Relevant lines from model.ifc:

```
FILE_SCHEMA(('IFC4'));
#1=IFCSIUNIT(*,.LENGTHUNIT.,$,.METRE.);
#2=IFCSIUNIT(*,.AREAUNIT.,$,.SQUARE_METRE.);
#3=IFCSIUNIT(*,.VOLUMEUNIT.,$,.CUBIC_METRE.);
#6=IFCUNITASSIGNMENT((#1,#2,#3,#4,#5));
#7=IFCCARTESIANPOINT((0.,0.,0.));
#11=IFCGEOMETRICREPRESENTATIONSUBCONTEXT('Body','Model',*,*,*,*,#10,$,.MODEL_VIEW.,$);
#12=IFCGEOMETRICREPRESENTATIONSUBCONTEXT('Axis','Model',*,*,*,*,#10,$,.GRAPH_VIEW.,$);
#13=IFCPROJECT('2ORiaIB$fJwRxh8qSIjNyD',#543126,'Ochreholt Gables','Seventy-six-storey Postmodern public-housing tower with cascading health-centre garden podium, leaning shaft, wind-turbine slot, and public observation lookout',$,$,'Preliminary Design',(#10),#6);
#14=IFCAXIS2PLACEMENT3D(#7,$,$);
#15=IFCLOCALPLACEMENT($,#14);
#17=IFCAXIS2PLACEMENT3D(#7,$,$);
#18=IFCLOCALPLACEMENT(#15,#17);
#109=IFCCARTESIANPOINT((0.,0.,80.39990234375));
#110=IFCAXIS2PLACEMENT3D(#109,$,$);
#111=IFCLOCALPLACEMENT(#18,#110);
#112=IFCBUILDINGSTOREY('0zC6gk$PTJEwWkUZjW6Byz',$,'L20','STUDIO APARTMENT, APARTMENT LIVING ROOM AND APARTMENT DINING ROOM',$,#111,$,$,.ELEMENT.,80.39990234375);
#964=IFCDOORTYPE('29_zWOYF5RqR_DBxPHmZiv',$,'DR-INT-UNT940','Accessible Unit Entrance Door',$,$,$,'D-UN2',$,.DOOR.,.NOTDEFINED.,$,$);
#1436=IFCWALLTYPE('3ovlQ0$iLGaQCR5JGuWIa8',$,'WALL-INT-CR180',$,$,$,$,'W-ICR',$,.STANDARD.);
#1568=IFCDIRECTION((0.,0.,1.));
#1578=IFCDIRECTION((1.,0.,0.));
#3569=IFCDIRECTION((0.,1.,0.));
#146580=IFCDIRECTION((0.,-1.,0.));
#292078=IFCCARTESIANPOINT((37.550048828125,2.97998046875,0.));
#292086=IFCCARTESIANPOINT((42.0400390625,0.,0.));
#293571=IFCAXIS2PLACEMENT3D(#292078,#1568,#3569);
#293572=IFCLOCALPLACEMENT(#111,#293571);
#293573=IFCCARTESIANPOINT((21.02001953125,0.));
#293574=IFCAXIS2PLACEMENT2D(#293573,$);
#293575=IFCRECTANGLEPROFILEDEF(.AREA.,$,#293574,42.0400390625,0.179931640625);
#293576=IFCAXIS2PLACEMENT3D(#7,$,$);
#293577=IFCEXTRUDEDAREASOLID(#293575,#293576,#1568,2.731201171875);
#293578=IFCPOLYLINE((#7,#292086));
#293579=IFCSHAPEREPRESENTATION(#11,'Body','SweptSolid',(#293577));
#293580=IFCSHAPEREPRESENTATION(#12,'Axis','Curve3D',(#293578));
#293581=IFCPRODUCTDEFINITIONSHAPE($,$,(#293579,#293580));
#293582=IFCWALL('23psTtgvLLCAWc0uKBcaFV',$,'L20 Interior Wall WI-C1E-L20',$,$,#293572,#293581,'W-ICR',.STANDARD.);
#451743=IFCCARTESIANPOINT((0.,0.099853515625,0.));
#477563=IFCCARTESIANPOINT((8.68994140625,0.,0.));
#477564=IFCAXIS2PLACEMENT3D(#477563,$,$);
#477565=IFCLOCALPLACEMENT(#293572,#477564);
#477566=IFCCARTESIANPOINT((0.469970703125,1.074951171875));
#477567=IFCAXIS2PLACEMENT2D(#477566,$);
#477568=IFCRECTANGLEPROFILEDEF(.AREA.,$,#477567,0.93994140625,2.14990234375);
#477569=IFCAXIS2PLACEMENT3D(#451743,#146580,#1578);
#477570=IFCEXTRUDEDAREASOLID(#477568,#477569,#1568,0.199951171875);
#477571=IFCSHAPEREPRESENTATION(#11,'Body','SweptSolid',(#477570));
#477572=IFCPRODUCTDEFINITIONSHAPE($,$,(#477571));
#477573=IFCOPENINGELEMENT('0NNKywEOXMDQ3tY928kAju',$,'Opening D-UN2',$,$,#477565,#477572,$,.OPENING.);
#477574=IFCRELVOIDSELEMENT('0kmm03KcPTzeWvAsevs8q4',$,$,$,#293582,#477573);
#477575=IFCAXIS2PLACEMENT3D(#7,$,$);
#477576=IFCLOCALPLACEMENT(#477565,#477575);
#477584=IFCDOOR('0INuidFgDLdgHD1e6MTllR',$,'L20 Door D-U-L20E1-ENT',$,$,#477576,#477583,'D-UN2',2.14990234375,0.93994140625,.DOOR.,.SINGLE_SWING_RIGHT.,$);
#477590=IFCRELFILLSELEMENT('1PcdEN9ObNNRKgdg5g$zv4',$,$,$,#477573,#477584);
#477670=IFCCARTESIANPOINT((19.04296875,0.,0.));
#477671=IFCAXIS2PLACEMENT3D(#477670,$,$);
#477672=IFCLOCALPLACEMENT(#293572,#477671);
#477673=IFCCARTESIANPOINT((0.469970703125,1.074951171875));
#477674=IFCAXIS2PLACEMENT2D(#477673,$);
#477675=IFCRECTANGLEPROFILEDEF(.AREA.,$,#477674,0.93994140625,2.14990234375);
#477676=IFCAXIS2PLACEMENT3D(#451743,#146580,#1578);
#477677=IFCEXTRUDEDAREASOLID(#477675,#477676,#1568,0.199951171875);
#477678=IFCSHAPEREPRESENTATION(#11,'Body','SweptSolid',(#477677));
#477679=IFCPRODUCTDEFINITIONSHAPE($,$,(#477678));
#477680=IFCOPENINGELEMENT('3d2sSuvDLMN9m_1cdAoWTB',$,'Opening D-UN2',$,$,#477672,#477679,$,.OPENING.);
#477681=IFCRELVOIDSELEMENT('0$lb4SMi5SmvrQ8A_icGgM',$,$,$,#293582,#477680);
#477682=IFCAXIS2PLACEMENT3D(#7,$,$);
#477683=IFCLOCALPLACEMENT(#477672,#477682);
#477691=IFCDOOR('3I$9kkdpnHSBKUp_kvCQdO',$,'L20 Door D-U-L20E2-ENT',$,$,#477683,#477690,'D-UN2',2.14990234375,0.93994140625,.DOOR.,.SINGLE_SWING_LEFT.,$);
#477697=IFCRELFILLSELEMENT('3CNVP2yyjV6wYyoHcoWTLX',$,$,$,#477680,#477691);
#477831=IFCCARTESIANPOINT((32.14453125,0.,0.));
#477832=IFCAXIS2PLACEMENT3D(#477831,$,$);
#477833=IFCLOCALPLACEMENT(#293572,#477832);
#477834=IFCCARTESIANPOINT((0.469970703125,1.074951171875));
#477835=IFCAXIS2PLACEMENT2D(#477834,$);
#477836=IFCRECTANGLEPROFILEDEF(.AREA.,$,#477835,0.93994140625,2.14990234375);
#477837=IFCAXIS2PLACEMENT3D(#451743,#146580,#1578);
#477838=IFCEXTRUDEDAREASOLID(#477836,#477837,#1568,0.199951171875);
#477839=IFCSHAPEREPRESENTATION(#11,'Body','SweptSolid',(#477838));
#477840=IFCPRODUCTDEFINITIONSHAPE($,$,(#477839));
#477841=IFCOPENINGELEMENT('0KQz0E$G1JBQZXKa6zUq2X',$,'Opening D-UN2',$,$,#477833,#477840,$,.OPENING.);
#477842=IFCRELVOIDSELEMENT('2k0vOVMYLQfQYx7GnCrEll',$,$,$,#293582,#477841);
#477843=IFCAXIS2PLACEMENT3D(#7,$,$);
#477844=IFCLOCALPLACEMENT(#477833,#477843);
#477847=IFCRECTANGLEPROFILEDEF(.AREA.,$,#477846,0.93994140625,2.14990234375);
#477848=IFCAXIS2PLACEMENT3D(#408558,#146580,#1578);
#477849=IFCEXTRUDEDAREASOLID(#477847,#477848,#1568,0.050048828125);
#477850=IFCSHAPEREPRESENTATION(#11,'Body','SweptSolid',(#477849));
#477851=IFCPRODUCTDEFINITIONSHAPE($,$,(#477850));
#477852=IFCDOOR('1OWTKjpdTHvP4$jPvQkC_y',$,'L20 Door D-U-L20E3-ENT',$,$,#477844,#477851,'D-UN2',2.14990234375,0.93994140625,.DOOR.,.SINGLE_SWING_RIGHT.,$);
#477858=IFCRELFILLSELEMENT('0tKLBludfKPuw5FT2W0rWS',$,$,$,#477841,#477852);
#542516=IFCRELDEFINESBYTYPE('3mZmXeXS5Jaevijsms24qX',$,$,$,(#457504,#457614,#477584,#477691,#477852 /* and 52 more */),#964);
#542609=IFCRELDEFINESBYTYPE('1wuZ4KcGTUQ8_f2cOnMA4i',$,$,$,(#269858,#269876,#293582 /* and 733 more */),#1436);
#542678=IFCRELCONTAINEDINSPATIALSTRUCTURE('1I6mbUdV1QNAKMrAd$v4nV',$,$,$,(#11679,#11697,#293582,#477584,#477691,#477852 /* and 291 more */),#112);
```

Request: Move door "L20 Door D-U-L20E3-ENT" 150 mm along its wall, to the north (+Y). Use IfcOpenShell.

```python
import ifcopenshell
import ifcopenshell.api.geometry
import ifcopenshell.util.placement

model = ifcopenshell.open("model.ifc")

door = model.by_id(477852)
opening = door.FillsVoids[0].RelatingOpeningElement
wall = opening.VoidsElements[0].RelatingBuildingElement

wall_matrix = ifcopenshell.util.placement.get_local_placement(wall.ObjectPlacement)
shift = wall_matrix[:3, 0] * 0.15
before = ifcopenshell.util.placement.get_local_placement(door.ObjectPlacement)[:3, 3].copy()

# The door is placed relative to its opening, so it follows when the opening moves.
matrix = ifcopenshell.util.placement.get_local_placement(opening.ObjectPlacement)
matrix[:3, 3] += shift
ifcopenshell.api.geometry.edit_object_placement(
    model, product=opening, matrix=matrix, is_si=False, should_transform_children=True
)

after = ifcopenshell.util.placement.get_local_placement(door.ObjectPlacement)[:3, 3]
print("door moved by", (after - before).round(3) + 0.0)

model.write("model-out.ifc")
```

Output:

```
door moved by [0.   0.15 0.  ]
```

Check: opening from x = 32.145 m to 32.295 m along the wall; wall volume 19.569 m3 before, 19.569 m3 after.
